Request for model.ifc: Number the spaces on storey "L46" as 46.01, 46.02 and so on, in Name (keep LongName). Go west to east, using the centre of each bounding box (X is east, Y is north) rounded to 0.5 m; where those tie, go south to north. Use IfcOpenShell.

First a look at what the model holds.

```python
import ifcopenshell
import ifcopenshell.util.element
import ifcopenshell.util.placement

model = ifcopenshell.open("model.ifc")
print(model.schema)
storey = next(s for s in model.by_type("IfcBuildingStorey") if s.Name == "L46")
spaces = [e for e in ifcopenshell.util.element.get_decomposition(storey) if e.is_a("IfcSpace")]
for e in sorted(spaces, key=lambda e: e.id()):
    origin = ifcopenshell.util.placement.get_local_placement(e.ObjectPlacement)[:3, 3]
    print(e.id(), e.Name, e.LongName, origin.round(2) + 0.0, sep=" | ")
```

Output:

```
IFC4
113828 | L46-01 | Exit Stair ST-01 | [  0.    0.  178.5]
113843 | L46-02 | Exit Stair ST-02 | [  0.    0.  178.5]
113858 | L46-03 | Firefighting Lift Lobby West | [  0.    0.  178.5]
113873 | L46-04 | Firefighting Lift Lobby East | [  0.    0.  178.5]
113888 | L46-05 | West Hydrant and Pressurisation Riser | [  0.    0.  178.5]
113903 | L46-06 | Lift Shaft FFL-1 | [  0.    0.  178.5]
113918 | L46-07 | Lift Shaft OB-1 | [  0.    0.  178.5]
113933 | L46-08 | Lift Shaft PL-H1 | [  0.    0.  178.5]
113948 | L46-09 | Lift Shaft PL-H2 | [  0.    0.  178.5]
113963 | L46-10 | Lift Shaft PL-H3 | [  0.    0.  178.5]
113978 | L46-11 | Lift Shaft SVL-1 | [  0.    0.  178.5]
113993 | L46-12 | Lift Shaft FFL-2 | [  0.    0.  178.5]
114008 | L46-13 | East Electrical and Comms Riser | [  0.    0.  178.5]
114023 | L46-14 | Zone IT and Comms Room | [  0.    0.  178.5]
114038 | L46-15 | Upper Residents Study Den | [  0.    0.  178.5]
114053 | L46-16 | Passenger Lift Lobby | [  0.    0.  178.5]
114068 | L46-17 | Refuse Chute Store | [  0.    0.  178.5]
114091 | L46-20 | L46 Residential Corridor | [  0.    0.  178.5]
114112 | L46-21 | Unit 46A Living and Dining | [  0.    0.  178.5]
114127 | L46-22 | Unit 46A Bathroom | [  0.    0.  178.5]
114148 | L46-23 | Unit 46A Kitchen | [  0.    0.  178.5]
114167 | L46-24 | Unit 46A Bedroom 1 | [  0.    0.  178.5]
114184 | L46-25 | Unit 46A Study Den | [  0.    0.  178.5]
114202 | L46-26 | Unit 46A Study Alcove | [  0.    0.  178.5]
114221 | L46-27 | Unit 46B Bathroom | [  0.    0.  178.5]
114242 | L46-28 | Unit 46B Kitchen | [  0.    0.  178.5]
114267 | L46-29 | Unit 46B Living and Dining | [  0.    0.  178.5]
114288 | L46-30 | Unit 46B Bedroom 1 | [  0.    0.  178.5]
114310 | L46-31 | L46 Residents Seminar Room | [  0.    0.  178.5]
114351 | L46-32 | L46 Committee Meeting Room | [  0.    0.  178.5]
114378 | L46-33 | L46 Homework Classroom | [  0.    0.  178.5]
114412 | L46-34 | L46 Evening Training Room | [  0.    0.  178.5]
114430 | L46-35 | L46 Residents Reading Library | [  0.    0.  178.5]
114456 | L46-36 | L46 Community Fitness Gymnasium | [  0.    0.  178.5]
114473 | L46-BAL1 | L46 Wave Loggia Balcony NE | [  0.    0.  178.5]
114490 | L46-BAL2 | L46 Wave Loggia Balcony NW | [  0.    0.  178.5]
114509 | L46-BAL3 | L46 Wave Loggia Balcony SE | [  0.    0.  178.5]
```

```python
import ifcopenshell
import ifcopenshell.geom
import ifcopenshell.util.element
import ifcopenshell.util.shape

model = ifcopenshell.open("model.ifc")
settings = ifcopenshell.geom.settings()
settings.set("use-world-coords", True)


def centre(element):
    shape = ifcopenshell.geom.create_shape(settings, element)
    return ifcopenshell.util.shape.get_bbox_centroid(shape.geometry)


storey = next(s for s in model.by_type("IfcBuildingStorey") if s.Name == "L46")
spaces = [e for e in ifcopenshell.util.element.get_decomposition(storey) if e.is_a("IfcSpace")]

# Insertion points can sit at a corner or the storey origin, so sort by the geometry (in metres).
centres = {e: centre(e) for e in spaces}
spaces.sort(key=lambda e: (round(centres[e][0] / 0.5), centres[e][1]))

for i, e in enumerate(spaces, start=1):
    number = f"46.{i:02d}"
    e.Name = number
    print(e.id(), number)

model.write("model_rev.ifc")
```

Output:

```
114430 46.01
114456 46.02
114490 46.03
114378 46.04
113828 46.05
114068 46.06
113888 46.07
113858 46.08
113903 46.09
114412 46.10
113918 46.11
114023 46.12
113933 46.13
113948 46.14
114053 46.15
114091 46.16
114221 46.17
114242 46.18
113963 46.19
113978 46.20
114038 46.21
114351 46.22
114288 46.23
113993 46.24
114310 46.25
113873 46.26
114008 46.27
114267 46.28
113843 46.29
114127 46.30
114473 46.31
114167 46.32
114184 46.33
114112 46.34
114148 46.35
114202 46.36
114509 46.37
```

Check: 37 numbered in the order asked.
